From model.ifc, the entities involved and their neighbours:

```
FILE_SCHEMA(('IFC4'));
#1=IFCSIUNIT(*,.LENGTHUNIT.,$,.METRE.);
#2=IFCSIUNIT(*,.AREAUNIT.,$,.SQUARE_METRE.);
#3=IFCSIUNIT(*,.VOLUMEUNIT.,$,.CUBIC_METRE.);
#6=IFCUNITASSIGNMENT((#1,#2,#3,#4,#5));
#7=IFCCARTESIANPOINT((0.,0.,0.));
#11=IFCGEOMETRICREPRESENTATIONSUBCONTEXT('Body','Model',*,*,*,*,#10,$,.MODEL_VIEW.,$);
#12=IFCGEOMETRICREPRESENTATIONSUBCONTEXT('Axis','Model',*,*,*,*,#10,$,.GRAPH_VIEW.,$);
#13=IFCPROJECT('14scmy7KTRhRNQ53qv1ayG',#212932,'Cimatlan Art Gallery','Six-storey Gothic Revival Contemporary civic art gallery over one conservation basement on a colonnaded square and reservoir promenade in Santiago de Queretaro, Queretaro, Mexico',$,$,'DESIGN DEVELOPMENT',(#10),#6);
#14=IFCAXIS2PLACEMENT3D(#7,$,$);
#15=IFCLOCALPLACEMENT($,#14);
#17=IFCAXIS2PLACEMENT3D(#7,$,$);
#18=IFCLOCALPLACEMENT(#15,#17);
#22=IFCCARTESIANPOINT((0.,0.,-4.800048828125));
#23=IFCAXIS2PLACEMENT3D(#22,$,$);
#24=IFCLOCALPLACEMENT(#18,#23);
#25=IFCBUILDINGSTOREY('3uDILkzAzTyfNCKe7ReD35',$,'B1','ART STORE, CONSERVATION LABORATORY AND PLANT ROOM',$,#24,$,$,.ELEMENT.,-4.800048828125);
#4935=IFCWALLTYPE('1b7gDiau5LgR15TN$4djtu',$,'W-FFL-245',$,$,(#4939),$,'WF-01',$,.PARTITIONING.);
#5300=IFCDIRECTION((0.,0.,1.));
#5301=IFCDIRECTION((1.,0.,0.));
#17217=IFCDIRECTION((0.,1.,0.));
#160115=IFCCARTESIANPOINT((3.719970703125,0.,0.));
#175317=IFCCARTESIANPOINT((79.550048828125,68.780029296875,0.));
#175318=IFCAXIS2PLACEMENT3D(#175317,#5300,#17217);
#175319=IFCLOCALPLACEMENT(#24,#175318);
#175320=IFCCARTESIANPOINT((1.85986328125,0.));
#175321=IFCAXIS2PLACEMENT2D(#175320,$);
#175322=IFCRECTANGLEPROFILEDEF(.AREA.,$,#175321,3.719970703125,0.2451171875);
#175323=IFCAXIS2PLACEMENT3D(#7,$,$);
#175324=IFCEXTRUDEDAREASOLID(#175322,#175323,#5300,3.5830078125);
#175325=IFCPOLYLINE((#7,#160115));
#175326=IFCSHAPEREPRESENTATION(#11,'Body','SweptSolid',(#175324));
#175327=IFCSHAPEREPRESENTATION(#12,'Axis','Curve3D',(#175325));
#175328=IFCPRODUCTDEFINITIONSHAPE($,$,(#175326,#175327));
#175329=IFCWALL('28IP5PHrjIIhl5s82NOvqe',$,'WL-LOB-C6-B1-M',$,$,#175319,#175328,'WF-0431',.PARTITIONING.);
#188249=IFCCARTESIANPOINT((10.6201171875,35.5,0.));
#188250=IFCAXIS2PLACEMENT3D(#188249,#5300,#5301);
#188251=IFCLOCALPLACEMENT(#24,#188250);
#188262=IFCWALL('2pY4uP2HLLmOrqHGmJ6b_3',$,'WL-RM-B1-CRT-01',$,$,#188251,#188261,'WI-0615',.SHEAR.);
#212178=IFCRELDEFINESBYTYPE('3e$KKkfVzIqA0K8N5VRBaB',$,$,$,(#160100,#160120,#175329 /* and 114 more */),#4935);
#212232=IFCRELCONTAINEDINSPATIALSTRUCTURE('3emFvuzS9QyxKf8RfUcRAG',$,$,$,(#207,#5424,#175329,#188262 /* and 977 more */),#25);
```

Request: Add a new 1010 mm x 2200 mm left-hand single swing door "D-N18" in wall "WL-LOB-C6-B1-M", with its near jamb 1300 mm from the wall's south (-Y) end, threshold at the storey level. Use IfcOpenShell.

```python
import numpy as np
import ifcopenshell
import ifcopenshell.api.feature
import ifcopenshell.api.geometry
import ifcopenshell.api.root
import ifcopenshell.api.spatial
import ifcopenshell.geom
import ifcopenshell.util.element
import ifcopenshell.util.placement
import ifcopenshell.util.representation
import ifcopenshell.util.shape
import ifcopenshell.util.unit

model = ifcopenshell.open("model.ifc")
unit_scale = ifcopenshell.util.unit.calculate_unit_scale(model)
settings = ifcopenshell.geom.settings()


def volume(element):
    """Net volume in cubic metres, openings subtracted."""
    shape = ifcopenshell.geom.create_shape(settings, element)
    return ifcopenshell.util.shape.get_volume(shape.geometry)


wall = model.by_id(175329)
storey = ifcopenshell.util.element.get_container(wall, ifc_class="IfcBuildingStorey")
context = ifcopenshell.util.representation.get_context(model, "Model", "Body", "MODEL_VIEW")
before = volume(wall)

width, height, from_end, sill = 1.01, 2.2, 1.3, 0.0  # metres

# The wall runs along its own X axis, and the end named is its -X end.
wall_shape = ifcopenshell.geom.create_shape(settings, wall)
x, y, z = ifcopenshell.util.shape.get_vertices(wall_shape.geometry).T
start = x.min() + from_end
face, thickness = float(y.min()), float(y.max() - y.min())
wall_matrix = ifcopenshell.util.placement.get_local_placement(wall.ObjectPlacement)
level = ifcopenshell.util.placement.get_local_placement(storey.ObjectPlacement)[2, 3]


def in_wall(x, y):
    """Placement at x, y metres in the wall's axes, at sill height."""
    matrix = wall_matrix.copy()
    matrix[:, 3] = wall_matrix @ np.array([x / unit_scale, y / unit_scale, 0.0, 1.0])
    matrix[2, 3] = level + sill / unit_scale
    return matrix


# Opening: a box that overshoots both wall faces by 50 mm.
opening = ifcopenshell.api.root.create_entity(model, ifc_class="IfcOpeningElement", predefined_type="OPENING")
box = ifcopenshell.api.geometry.add_wall_representation(
    model, context=context, length=width, height=height, thickness=thickness + 0.1
)
ifcopenshell.api.geometry.assign_representation(model, product=opening, representation=box)
ifcopenshell.api.geometry.edit_object_placement(model, product=opening, matrix=in_wall(start, face - 0.05), is_si=False)
ifcopenshell.api.feature.add_feature(model, feature=opening, element=wall)

door = ifcopenshell.api.root.create_entity(model, ifc_class="IfcDoor", name="D-N18", predefined_type="DOOR")
door.OverallWidth, door.OverallHeight = width / unit_scale, height / unit_scale
door.OperationType = "SINGLE_SWING_LEFT"
body = ifcopenshell.api.geometry.add_door_representation(
    model,
    context=context,
    overall_width=door.OverallWidth,
    overall_height=door.OverallHeight,
    operation_type="SINGLE_SWING_LEFT",
    lining_properties={"LiningDepth": thickness / unit_scale, "ThresholdDepth": thickness / unit_scale},
)
ifcopenshell.api.geometry.assign_representation(model, product=door, representation=body)
ifcopenshell.api.spatial.assign_container(model, products=[door], relating_structure=storey)
ifcopenshell.api.feature.add_filling(model, opening=opening, element=door)

# The lining spans the wall, so the door starts at the wall face.
ifcopenshell.api.geometry.edit_object_placement(model, product=door, matrix=in_wall(start, face), is_si=False)

after = volume(wall)

print(f"wall volume {before:.3f} -> {after:.3f} m3")

model.write("model-out.ifc")
```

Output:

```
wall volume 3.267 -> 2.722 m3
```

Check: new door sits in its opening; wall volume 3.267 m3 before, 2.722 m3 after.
